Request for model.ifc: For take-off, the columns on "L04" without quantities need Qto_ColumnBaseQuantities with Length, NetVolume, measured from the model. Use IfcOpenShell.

First a look at what the model holds.

```python
import ifcopenshell
import ifcopenshell.util.element
import ifcopenshell.util.unit

model = ifcopenshell.open("model.ifc")
print(model.schema)
for unit_type in ("LENGTHUNIT", "AREAUNIT", "VOLUMEUNIT"):
    print(unit_type, ifcopenshell.util.unit.calculate_unit_scale(model, unit_type))
storey = next(s for s in model.by_type("IfcBuildingStorey") if s.Name == "L04")
columns = [e for e in ifcopenshell.util.element.get_decomposition(storey) if e.is_a("IfcColumn")]
for e in sorted(columns, key=lambda e: e.id()):
    print(e.id(), e.is_a(), e.Name, list(ifcopenshell.util.element.get_psets(e, qtos_only=True)), sep=" | ")
```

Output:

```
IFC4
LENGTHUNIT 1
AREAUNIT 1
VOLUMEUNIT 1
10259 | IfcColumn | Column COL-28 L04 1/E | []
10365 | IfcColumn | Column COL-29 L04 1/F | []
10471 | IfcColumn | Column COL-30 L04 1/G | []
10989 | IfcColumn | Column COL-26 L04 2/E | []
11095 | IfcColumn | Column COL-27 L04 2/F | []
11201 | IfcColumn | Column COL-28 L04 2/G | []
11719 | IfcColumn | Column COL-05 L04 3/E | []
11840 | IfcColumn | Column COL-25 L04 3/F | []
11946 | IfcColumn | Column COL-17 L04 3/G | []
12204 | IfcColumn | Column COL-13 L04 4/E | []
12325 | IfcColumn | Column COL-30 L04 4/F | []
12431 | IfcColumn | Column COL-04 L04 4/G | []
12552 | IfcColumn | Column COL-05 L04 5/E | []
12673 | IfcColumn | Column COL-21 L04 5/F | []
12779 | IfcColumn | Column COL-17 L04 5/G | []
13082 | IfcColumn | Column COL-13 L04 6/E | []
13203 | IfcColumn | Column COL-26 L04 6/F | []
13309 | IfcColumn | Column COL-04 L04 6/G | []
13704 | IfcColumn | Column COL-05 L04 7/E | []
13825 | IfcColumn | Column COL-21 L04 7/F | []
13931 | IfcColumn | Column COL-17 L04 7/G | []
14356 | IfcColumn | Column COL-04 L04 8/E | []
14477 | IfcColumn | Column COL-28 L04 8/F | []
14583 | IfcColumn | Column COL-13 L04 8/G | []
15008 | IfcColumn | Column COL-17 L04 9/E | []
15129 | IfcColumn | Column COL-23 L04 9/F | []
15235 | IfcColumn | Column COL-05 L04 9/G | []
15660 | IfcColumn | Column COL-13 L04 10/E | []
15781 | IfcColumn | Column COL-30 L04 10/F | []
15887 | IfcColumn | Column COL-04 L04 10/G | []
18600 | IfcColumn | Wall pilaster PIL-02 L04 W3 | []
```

```python
import ifcopenshell
import ifcopenshell.api.pset
import ifcopenshell.geom
import ifcopenshell.util.element
import ifcopenshell.util.shape
import ifcopenshell.util.unit

model = ifcopenshell.open("model.ifc")
unit_scale = ifcopenshell.util.unit.calculate_unit_scale(model)
volume_scale = ifcopenshell.util.unit.calculate_unit_scale(model, "VOLUMEUNIT")
settings = ifcopenshell.geom.settings()

storey = next(s for s in model.by_type("IfcBuildingStorey") if s.Name == "L04")
columns = [e for e in ifcopenshell.util.element.get_decomposition(storey) if e.is_a("IfcColumn")]

for e in sorted(columns, key=lambda e: e.id()):
    if ifcopenshell.util.element.get_psets(e, qtos_only=True, should_inherit=False):
        continue
    # Geometry comes back in metres, in the element's own axes.
    shape = ifcopenshell.geom.create_shape(settings, e)
    values = {
        "Length": ifcopenshell.util.shape.get_z(shape.geometry) / unit_scale,
        "NetVolume": ifcopenshell.util.shape.get_volume(shape.geometry) / volume_scale,
    }
    qto = ifcopenshell.api.pset.add_qto(model, product=e, name="Qto_ColumnBaseQuantities")
    ifcopenshell.api.pset.edit_qto(model, qto=qto, properties=values)
    print(e.id(), {k: round(v, 3) for k, v in values.items()})

model.write("model_edited.ifc")
```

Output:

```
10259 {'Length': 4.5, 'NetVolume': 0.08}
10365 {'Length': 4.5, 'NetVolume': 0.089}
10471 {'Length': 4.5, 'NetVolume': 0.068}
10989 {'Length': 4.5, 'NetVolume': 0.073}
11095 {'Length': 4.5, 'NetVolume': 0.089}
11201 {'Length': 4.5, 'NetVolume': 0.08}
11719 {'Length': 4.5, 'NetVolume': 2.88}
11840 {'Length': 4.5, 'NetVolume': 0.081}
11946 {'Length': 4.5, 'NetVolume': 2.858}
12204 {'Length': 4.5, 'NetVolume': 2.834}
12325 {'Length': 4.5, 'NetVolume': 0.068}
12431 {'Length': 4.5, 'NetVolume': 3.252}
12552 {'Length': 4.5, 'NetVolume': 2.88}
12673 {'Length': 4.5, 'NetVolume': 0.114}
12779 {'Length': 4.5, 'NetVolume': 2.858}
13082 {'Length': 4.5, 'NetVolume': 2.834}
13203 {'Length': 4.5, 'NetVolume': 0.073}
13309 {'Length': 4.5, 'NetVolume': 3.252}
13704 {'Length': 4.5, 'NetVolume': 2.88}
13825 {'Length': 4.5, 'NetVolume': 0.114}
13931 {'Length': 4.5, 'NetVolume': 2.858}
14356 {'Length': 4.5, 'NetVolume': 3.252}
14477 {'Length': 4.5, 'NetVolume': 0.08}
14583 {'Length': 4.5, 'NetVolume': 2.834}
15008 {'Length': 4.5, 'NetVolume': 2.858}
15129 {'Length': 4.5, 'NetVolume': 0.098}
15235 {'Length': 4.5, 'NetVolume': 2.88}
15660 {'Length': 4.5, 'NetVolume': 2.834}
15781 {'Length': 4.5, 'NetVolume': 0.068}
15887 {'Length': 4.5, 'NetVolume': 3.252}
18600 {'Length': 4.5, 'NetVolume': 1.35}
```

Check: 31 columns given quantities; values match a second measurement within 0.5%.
